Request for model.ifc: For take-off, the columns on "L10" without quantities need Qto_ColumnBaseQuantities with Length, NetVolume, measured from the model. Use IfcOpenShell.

First a look at what the model holds.

```python
import ifcopenshell
import ifcopenshell.util.element
import ifcopenshell.util.unit

model = ifcopenshell.open("model.ifc")
print(model.schema)
for unit_type in ("LENGTHUNIT", "AREAUNIT", "VOLUMEUNIT"):
    print(unit_type, ifcopenshell.util.unit.calculate_unit_scale(model, unit_type))
storey = next(s for s in model.by_type("IfcBuildingStorey") if s.Name == "L10")
columns = [e for e in ifcopenshell.util.element.get_decomposition(storey) if e.is_a("IfcColumn")]
for e in sorted(columns, key=lambda e: e.id()):
    print(e.id(), e.is_a(), e.Name, list(ifcopenshell.util.element.get_psets(e, qtos_only=True)), sep=" | ")
```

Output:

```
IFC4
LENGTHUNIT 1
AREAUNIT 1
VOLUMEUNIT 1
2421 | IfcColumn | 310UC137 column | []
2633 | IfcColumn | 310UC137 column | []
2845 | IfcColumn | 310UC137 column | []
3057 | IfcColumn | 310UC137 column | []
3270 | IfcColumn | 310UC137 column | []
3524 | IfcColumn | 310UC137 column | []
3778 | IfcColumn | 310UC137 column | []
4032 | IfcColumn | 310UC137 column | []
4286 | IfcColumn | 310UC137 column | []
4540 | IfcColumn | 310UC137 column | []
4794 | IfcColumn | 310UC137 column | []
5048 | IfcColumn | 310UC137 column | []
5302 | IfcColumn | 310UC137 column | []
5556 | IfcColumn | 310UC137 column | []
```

```python
import ifcopenshell
import ifcopenshell.api.pset
import ifcopenshell.geom
import ifcopenshell.util.element
import ifcopenshell.util.shape
import ifcopenshell.util.unit

model = ifcopenshell.open("model.ifc")
unit_scale = ifcopenshell.util.unit.calculate_unit_scale(model)
volume_scale = ifcopenshell.util.unit.calculate_unit_scale(model, "VOLUMEUNIT")
settings = ifcopenshell.geom.settings()

storey = next(s for s in model.by_type("IfcBuildingStorey") if s.Name == "L10")
columns = [e for e in ifcopenshell.util.element.get_decomposition(storey) if e.is_a("IfcColumn")]

for e in sorted(columns, key=lambda e: e.id()):
    if ifcopenshell.util.element.get_psets(e, qtos_only=True, should_inherit=False):
        continue
    # Geometry comes back in metres, in the element's own axes.
    shape = ifcopenshell.geom.create_shape(settings, e)
    values = {
        "Length": ifcopenshell.util.shape.get_z(shape.geometry) / unit_scale,
        "NetVolume": ifcopenshell.util.shape.get_volume(shape.geometry) / volume_scale,
    }
    qto = ifcopenshell.api.pset.add_qto(model, product=e, name="Qto_ColumnBaseQuantities")
    ifcopenshell.api.pset.edit_qto(model, qto=qto, properties=values)
    print(e.id(), {k: round(v, 3) for k, v in values.items()})

model.write("model_rev.ifc")
```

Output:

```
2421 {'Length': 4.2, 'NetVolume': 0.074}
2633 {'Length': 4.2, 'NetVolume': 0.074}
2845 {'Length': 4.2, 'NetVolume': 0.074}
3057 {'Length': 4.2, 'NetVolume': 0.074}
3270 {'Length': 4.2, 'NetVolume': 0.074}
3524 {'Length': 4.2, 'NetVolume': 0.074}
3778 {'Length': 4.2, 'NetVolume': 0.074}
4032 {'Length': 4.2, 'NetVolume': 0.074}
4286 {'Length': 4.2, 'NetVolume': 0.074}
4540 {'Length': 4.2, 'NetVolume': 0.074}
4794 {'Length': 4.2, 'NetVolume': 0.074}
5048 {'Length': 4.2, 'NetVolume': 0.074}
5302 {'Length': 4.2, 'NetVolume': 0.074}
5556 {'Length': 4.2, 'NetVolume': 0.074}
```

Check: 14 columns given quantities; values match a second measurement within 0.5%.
